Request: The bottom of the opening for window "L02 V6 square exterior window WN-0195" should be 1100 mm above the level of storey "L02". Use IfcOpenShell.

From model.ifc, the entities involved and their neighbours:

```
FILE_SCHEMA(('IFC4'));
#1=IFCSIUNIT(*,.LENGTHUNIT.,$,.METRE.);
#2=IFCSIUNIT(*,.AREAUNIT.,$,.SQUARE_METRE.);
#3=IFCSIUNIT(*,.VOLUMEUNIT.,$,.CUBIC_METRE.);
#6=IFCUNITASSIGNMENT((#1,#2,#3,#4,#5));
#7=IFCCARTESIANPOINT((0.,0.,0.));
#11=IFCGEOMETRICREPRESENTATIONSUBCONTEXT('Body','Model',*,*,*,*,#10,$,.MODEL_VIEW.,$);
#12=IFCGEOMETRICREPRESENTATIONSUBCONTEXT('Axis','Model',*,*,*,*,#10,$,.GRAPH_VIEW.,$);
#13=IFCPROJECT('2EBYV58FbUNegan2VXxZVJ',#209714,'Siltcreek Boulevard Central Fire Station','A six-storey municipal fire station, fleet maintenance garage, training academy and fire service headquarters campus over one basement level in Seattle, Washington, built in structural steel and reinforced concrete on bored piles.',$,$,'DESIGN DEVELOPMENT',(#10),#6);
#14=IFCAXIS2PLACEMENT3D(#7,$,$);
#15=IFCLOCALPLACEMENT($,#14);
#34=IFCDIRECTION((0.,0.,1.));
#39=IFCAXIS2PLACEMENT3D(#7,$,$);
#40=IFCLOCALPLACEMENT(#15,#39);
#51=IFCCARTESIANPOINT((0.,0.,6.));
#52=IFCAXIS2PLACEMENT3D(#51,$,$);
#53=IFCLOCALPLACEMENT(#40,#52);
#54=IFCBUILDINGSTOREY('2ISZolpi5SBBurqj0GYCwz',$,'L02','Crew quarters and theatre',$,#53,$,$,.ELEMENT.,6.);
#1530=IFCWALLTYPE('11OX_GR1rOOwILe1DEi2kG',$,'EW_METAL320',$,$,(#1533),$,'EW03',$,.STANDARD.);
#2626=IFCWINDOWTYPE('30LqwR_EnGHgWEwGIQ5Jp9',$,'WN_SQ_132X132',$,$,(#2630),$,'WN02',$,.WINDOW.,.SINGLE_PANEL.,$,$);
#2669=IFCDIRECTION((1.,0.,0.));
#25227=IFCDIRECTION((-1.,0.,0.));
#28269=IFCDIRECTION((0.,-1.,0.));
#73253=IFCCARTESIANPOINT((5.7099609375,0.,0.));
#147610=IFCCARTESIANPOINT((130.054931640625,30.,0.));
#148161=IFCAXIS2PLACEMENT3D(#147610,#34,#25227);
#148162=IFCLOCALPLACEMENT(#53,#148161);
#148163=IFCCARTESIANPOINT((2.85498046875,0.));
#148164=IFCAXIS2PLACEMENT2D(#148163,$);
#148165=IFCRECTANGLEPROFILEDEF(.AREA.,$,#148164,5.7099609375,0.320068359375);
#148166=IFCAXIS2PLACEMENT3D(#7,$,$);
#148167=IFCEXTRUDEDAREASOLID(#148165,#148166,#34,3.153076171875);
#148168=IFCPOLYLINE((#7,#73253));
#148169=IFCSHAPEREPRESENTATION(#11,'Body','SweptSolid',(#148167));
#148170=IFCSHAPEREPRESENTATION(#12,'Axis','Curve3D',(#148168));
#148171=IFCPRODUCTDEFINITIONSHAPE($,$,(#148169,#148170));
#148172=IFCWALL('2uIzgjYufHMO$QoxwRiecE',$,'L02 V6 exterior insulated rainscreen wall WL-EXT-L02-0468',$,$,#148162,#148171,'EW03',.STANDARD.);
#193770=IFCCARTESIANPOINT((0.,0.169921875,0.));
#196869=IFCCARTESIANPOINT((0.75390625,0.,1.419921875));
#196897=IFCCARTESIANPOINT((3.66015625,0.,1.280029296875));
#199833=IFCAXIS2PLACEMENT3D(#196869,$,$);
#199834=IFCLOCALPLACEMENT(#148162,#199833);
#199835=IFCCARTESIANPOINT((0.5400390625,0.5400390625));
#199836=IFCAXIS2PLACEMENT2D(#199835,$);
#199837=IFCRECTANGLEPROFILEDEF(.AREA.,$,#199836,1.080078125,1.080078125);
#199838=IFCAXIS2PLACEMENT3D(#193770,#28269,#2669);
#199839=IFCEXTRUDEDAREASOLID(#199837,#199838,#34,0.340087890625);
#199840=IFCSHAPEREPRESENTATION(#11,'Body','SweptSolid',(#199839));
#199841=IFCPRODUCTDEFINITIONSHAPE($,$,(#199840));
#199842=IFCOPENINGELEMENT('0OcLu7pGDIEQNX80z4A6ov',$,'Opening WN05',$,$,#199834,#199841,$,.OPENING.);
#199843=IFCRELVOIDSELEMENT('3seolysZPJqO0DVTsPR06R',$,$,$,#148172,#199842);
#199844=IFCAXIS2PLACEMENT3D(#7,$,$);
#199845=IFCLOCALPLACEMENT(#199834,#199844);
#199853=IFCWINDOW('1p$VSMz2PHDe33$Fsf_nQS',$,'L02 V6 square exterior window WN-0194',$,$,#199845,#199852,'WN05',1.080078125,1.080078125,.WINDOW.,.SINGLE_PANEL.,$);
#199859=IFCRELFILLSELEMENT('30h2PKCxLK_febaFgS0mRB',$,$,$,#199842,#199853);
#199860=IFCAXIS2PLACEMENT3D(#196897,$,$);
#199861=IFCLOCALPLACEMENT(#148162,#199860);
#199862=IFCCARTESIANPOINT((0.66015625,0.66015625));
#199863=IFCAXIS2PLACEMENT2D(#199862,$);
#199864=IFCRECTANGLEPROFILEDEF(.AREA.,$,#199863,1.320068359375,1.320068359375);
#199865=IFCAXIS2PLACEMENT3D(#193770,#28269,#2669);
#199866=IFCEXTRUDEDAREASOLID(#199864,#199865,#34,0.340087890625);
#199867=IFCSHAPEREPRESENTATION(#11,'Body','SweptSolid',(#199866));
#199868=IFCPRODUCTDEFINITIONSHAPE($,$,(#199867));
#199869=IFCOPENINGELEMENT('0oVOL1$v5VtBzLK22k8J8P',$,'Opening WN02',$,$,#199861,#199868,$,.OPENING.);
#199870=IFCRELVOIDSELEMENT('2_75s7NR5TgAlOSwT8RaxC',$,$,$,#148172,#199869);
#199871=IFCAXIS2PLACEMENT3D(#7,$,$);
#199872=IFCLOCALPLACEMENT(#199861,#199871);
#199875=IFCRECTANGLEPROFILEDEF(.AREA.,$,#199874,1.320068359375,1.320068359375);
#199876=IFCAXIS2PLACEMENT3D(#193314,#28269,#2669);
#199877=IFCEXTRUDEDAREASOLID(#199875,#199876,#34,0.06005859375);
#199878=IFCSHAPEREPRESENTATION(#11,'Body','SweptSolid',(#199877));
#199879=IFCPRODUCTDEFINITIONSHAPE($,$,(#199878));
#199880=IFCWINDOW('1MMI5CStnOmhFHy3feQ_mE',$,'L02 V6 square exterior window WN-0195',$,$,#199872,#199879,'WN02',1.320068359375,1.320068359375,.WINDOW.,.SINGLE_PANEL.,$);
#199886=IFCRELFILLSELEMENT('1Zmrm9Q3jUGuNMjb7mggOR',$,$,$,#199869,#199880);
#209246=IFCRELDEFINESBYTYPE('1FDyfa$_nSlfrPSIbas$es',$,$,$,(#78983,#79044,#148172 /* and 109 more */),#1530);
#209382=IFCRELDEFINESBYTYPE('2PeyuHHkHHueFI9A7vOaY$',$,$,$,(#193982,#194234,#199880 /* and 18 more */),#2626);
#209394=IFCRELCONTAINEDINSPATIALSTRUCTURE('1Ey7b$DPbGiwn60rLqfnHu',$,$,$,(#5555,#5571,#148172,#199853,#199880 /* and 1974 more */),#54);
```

```python
import numpy as np
import ifcopenshell
import ifcopenshell.api.geometry
import ifcopenshell.geom
import ifcopenshell.util.element
import ifcopenshell.util.placement
import ifcopenshell.util.shape
import ifcopenshell.util.unit

model = ifcopenshell.open("model.ifc")
unit_scale = ifcopenshell.util.unit.calculate_unit_scale(model)

window = model.by_id(199880)
opening = window.FillsVoids[0].RelatingOpeningElement
storey = ifcopenshell.util.element.get_container(window, ifc_class="IfcBuildingStorey")
level = ifcopenshell.util.placement.get_local_placement(storey.ObjectPlacement)[2, 3]

# The opening's origin need not be at the sill, so measure its lowest point.
shape = ifcopenshell.geom.create_shape(ifcopenshell.geom.settings(), opening)
bottom = ifcopenshell.util.shape.get_shape_bottom_elevation(shape, shape.geometry) / unit_scale
dz = level + 1.1 - bottom

shift = np.array([0.0, 0.0, dz])
# The window is placed relative to its opening, so it follows when the opening moves.
matrix = ifcopenshell.util.placement.get_local_placement(opening.ObjectPlacement)
matrix[:3, 3] += shift
ifcopenshell.api.geometry.edit_object_placement(
    model, product=opening, matrix=matrix, is_si=False, should_transform_children=True
)

print(f"moved by {dz * unit_scale:+.3f} m")

model.write("model_v2.ifc")
```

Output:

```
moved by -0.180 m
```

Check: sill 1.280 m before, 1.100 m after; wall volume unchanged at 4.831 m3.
